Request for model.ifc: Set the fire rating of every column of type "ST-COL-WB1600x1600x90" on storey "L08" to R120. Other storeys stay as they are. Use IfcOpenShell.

First a look at what the model holds.

```python
import ifcopenshell
import ifcopenshell.util.element

model = ifcopenshell.open("model.ifc")
print(model.schema)
storey = next(s for s in model.by_type("IfcBuildingStorey") if s.Name == "L08")
columns = [e for e in ifcopenshell.util.element.get_decomposition(storey) if e.is_a("IfcColumn")]
seen = {}
for e in columns:
    element_type = ifcopenshell.util.element.get_type(e)
    key = (element_type.Name if element_type != e and element_type else None, ifcopenshell.util.element.get_pset(e, "Pset_ColumnCommon", "FireRating"))
    seen[key] = seen.get(key, 0) + 1
for (name, value), count in sorted(seen.items(), key=str):
    print(count, "x", name, "|", value)
```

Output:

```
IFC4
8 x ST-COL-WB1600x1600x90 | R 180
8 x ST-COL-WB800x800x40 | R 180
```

```python
import ifcopenshell
import ifcopenshell.api.pset
import ifcopenshell.util.element

model = ifcopenshell.open("model.ifc")

storey = next(s for s in model.by_type("IfcBuildingStorey") if s.Name == "L08")
columns = [e for e in ifcopenshell.util.element.get_decomposition(storey) if e.is_a("IfcColumn")]

count = 0
for e in columns:
    element_type = ifcopenshell.util.element.get_type(e)
    if element_type in (None, e) or element_type.Name != "ST-COL-WB1600x1600x90":
        continue
    found = ifcopenshell.util.element.get_pset(e, "Pset_ColumnCommon", should_inherit=False)
    if found:
        pset = model.by_id(found["id"])
        if len(ifcopenshell.util.element.get_elements_by_pset(pset)) > 1:
            pset = ifcopenshell.api.pset.unshare_pset(model, products=[e], pset=pset)[0]
    else:
        pset = ifcopenshell.api.pset.add_pset(model, product=e, name="Pset_ColumnCommon")
    ifcopenshell.api.pset.edit_pset(model, pset=pset, properties={"FireRating": "R120"})
    count += 1

print(count, "columns updated")

model.write("model-out.ifc")
```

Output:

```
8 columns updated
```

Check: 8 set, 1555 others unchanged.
